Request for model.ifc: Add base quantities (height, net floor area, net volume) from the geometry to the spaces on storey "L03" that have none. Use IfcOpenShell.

First a look at what the model holds.

```python
import ifcopenshell
import ifcopenshell.util.element
import ifcopenshell.util.unit

model = ifcopenshell.open("model.ifc")
print(model.schema)
for unit_type in ("LENGTHUNIT", "AREAUNIT", "VOLUMEUNIT"):
    print(unit_type, ifcopenshell.util.unit.calculate_unit_scale(model, unit_type))
storey = next(s for s in model.by_type("IfcBuildingStorey") if s.Name == "L03")
spaces = [e for e in ifcopenshell.util.element.get_decomposition(storey) if e.is_a("IfcSpace")]
for e in sorted(spaces, key=lambda e: e.id()):
    print(e.id(), e.is_a(), e.Name, list(ifcopenshell.util.element.get_psets(e, qtos_only=True)), sep=" | ")
```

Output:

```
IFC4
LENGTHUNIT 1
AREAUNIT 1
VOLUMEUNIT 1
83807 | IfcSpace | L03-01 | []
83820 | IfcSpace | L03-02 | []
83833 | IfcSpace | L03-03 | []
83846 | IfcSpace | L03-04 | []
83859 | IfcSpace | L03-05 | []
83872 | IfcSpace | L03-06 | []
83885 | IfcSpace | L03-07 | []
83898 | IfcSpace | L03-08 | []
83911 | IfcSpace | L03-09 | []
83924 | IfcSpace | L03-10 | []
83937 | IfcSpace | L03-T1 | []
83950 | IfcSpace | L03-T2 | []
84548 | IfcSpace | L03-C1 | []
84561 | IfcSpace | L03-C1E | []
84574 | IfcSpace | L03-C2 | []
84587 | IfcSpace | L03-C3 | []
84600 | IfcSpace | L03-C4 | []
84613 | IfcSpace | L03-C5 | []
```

```python
import ifcopenshell
import ifcopenshell.api.pset
import ifcopenshell.geom
import ifcopenshell.util.element
import ifcopenshell.util.shape
import ifcopenshell.util.unit

model = ifcopenshell.open("model.ifc")
unit_scale = ifcopenshell.util.unit.calculate_unit_scale(model)
area_scale = ifcopenshell.util.unit.calculate_unit_scale(model, "AREAUNIT")
volume_scale = ifcopenshell.util.unit.calculate_unit_scale(model, "VOLUMEUNIT")
settings = ifcopenshell.geom.settings()

storey = next(s for s in model.by_type("IfcBuildingStorey") if s.Name == "L03")
spaces = [e for e in ifcopenshell.util.element.get_decomposition(storey) if e.is_a("IfcSpace")]

for e in sorted(spaces, key=lambda e: e.id()):
    if ifcopenshell.util.element.get_psets(e, qtos_only=True, should_inherit=False):
        continue
    # Geometry comes back in metres, in the element's own axes.
    shape = ifcopenshell.geom.create_shape(settings, e)
    values = {
        "Height": ifcopenshell.util.shape.get_z(shape.geometry) / unit_scale,
        "NetFloorArea": ifcopenshell.util.shape.get_footprint_area(shape.geometry) / area_scale,
        "NetVolume": ifcopenshell.util.shape.get_volume(shape.geometry) / volume_scale,
    }
    qto = ifcopenshell.api.pset.add_qto(model, product=e, name="Qto_SpaceBaseQuantities")
    ifcopenshell.api.pset.edit_qto(model, qto=qto, properties=values)
    print(e.id(), {k: round(v, 3) for k, v in values.items()})

model.write("model_v2.ifc")
```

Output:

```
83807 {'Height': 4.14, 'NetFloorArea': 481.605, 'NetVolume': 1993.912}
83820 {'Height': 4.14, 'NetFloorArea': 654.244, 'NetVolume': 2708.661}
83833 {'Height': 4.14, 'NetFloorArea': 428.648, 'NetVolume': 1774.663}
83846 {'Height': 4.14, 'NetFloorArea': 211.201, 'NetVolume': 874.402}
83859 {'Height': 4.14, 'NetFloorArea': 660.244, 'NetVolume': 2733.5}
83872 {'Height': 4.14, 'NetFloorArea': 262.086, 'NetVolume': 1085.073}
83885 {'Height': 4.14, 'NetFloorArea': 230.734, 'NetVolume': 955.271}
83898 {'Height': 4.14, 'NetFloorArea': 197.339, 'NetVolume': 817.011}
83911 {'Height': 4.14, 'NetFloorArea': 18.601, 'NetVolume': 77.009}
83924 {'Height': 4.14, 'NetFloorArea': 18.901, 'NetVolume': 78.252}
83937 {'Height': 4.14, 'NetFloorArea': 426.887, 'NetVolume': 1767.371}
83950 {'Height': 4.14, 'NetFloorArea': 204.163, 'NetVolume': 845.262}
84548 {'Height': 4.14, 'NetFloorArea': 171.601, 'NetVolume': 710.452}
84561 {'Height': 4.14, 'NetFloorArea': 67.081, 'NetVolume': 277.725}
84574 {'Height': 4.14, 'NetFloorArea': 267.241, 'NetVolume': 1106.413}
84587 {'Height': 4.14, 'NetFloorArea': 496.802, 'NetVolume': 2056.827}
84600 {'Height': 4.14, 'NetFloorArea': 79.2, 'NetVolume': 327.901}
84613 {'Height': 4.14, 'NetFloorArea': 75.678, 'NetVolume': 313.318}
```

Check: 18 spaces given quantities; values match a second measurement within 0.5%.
